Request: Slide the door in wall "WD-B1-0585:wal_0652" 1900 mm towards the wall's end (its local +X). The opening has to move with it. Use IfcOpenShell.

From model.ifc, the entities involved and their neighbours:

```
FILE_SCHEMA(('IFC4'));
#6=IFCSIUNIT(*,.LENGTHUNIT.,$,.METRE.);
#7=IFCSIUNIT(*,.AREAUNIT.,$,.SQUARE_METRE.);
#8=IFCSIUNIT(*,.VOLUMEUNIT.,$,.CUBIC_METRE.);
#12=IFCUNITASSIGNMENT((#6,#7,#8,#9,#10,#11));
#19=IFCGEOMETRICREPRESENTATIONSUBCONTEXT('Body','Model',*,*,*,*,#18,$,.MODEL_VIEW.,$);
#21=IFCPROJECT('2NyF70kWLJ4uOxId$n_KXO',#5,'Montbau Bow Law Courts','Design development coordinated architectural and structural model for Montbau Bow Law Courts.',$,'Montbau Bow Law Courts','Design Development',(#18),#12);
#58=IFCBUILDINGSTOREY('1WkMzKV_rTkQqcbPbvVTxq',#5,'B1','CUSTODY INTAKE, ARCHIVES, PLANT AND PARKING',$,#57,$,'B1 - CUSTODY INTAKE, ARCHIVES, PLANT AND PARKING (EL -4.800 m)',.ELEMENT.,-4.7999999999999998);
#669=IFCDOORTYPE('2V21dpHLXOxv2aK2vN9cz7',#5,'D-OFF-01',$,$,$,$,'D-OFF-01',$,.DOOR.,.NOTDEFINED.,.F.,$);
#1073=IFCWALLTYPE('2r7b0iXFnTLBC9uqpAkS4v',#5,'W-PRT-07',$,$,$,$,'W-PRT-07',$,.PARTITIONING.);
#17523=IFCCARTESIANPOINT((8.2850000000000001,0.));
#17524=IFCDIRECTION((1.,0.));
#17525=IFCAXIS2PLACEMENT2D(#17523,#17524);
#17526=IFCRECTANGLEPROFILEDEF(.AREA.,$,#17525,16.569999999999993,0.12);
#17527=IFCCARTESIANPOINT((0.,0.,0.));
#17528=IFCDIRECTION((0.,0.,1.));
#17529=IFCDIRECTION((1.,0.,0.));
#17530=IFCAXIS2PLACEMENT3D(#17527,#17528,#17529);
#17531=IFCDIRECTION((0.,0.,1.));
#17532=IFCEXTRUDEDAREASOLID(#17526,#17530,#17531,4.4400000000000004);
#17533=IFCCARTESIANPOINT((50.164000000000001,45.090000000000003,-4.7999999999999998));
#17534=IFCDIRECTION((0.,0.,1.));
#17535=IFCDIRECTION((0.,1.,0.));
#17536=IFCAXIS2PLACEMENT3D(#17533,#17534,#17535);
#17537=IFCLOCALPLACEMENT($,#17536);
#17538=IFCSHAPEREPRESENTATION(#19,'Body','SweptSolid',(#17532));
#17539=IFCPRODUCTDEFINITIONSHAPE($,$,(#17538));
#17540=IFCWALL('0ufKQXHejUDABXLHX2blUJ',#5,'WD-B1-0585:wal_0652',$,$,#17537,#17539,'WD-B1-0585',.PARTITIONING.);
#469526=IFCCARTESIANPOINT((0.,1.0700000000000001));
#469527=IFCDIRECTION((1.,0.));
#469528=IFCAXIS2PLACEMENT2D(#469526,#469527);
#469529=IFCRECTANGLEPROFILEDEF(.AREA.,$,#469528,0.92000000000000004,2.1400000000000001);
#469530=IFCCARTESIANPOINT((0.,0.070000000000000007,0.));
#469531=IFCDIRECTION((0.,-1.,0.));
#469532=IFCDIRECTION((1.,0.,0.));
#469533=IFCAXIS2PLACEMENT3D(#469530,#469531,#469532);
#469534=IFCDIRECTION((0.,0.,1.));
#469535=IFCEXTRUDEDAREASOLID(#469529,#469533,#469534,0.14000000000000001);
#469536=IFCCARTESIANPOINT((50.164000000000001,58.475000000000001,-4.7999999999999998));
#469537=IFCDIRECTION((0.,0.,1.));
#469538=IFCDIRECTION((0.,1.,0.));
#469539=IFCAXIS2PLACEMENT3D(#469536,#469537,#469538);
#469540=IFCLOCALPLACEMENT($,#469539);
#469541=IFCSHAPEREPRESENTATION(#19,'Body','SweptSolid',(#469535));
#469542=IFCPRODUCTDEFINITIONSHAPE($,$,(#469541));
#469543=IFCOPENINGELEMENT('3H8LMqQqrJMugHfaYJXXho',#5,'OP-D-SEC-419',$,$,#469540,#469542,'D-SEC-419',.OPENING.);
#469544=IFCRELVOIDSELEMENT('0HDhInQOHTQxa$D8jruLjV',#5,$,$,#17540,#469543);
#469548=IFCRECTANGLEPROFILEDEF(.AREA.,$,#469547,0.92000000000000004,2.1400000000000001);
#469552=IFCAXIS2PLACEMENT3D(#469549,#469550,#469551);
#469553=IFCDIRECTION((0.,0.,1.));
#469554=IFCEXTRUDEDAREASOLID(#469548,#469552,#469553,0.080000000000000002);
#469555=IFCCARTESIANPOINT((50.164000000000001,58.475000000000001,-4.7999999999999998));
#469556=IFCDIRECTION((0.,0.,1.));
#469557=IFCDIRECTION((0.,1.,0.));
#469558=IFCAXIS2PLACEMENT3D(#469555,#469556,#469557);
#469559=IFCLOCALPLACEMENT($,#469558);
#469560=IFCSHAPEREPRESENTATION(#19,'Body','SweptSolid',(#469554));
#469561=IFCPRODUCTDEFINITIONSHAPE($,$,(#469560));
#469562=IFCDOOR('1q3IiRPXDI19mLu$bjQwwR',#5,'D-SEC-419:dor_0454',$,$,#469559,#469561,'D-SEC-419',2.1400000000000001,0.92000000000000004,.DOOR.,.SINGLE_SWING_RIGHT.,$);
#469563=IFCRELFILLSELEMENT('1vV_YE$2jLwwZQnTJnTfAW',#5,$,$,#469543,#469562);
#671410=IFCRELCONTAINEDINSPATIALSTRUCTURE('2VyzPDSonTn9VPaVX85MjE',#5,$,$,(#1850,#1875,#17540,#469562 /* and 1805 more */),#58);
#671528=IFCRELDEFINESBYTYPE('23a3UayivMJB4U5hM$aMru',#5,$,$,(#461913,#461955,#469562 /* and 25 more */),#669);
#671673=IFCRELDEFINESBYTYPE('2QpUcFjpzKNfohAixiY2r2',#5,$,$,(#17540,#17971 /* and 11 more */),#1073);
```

```python
import ifcopenshell
import ifcopenshell.api.geometry
import ifcopenshell.util.placement

model = ifcopenshell.open("model.ifc")

door = model.by_guid("1q3IiRPXDI19mLu$bjQwwR")
opening = door.FillsVoids[0].RelatingOpeningElement
wall = opening.VoidsElements[0].RelatingBuildingElement

wall_matrix = ifcopenshell.util.placement.get_local_placement(wall.ObjectPlacement)
shift = wall_matrix[:3, 0] * 1.9
before = ifcopenshell.util.placement.get_local_placement(door.ObjectPlacement)[:3, 3].copy()

# The door is not placed relative to its opening, so move both.
for product in (opening, door):
    matrix = ifcopenshell.util.placement.get_local_placement(product.ObjectPlacement)
    matrix[:3, 3] += shift
    ifcopenshell.api.geometry.edit_object_placement(model, product=product, matrix=matrix, is_si=False)

after = ifcopenshell.util.placement.get_local_placement(door.ObjectPlacement)[:3, 3]
print("door moved by", (after - before).round(3) + 0.0)

model.write("model_updated.ifc")
```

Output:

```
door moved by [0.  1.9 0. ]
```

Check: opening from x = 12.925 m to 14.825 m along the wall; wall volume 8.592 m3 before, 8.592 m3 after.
